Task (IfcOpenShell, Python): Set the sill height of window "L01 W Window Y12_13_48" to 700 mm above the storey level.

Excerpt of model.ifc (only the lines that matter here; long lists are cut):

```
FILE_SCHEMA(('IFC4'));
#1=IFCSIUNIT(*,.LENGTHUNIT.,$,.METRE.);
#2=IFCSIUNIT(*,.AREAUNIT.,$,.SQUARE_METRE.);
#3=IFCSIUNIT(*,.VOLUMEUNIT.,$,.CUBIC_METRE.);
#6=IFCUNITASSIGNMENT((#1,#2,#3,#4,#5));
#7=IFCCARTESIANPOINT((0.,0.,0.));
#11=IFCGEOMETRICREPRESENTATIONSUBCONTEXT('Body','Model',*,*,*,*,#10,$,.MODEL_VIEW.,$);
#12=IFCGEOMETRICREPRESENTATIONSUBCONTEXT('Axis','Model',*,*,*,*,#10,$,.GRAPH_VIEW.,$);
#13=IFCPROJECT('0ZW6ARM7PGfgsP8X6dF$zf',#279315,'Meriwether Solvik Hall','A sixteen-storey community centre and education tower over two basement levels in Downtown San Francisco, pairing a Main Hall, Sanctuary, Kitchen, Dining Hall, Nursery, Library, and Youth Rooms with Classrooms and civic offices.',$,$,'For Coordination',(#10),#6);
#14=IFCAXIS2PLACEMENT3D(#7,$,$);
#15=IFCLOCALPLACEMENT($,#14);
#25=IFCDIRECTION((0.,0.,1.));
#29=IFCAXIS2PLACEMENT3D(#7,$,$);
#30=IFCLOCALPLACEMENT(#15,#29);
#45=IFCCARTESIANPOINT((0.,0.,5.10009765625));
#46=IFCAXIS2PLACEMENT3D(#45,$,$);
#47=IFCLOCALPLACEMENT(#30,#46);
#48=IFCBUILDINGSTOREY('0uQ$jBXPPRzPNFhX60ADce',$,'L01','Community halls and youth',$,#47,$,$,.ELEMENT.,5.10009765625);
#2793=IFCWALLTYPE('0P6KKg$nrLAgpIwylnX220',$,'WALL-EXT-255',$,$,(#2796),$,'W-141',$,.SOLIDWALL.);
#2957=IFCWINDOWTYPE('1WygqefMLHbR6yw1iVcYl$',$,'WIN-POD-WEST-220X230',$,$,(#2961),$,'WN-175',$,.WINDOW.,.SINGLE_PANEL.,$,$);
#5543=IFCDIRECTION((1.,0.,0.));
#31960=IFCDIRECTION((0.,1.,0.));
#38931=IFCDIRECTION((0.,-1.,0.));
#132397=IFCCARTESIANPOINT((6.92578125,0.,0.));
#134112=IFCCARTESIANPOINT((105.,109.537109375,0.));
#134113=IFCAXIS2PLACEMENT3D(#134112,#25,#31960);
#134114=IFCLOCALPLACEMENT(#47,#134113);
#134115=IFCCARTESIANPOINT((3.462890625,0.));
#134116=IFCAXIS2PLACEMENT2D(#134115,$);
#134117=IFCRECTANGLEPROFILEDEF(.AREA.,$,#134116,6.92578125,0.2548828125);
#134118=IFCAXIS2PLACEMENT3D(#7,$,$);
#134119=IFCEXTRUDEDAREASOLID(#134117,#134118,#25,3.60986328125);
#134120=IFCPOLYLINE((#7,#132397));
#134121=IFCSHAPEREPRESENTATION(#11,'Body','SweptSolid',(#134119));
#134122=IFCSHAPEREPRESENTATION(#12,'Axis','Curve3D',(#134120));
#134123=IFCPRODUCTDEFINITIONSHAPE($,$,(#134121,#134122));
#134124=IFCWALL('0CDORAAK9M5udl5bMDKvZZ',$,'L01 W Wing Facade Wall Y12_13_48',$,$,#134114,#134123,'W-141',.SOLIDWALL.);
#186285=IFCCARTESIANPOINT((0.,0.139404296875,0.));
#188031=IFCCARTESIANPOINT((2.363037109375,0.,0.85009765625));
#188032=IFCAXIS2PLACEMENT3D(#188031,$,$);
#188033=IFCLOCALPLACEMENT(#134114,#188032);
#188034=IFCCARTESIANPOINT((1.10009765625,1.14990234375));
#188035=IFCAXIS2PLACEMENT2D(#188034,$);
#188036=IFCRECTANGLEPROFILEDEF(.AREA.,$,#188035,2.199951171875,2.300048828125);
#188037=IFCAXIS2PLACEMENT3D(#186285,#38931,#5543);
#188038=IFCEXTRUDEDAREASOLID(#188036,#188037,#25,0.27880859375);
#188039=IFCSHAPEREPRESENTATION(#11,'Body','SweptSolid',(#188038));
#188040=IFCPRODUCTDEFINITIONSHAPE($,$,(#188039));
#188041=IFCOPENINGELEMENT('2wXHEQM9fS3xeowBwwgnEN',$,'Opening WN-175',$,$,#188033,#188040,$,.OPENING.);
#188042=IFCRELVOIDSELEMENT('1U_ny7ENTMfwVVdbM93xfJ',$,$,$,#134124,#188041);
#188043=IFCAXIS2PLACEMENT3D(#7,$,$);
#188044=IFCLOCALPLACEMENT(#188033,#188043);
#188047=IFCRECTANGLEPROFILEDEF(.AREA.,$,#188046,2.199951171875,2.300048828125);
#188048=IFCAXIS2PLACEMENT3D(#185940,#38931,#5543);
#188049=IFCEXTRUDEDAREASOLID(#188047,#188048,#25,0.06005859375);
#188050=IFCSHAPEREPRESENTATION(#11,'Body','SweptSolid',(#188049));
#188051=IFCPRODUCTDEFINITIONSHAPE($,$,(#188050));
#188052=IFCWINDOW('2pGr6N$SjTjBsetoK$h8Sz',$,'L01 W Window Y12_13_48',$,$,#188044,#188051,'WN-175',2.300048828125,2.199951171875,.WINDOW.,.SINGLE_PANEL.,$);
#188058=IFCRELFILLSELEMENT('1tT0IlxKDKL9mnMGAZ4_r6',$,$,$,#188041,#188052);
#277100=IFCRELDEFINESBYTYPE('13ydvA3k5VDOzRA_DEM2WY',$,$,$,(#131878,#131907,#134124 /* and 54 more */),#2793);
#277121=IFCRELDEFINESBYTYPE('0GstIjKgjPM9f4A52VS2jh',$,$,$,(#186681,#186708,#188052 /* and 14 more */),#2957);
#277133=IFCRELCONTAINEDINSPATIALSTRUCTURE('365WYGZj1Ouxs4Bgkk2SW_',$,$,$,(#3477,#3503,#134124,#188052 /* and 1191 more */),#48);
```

```python
import numpy as np
import ifcopenshell
import ifcopenshell.api.geometry
import ifcopenshell.geom
import ifcopenshell.util.element
import ifcopenshell.util.placement
import ifcopenshell.util.shape
import ifcopenshell.util.unit

model = ifcopenshell.open("model.ifc")
unit_scale = ifcopenshell.util.unit.calculate_unit_scale(model)

window = model.by_guid("2pGr6N$SjTjBsetoK$h8Sz")
opening = window.FillsVoids[0].RelatingOpeningElement
storey = ifcopenshell.util.element.get_container(window, ifc_class="IfcBuildingStorey")
level = ifcopenshell.util.placement.get_local_placement(storey.ObjectPlacement)[2, 3]

# The opening's origin need not be at the sill, so measure its lowest point.
shape = ifcopenshell.geom.create_shape(ifcopenshell.geom.settings(), opening)
bottom = ifcopenshell.util.shape.get_shape_bottom_elevation(shape, shape.geometry) / unit_scale
dz = level + 0.7 - bottom

shift = np.array([0.0, 0.0, dz])
# The window is placed relative to its opening, so it follows when the opening moves.
matrix = ifcopenshell.util.placement.get_local_placement(opening.ObjectPlacement)
matrix[:3, 3] += shift
ifcopenshell.api.geometry.edit_object_placement(
    model, product=opening, matrix=matrix, is_si=False, should_transform_children=True
)

print(f"moved by {dz * unit_scale:+.3f} m")

model.write("model-out.ifc")
```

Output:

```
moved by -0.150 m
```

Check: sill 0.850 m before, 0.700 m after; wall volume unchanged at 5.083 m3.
